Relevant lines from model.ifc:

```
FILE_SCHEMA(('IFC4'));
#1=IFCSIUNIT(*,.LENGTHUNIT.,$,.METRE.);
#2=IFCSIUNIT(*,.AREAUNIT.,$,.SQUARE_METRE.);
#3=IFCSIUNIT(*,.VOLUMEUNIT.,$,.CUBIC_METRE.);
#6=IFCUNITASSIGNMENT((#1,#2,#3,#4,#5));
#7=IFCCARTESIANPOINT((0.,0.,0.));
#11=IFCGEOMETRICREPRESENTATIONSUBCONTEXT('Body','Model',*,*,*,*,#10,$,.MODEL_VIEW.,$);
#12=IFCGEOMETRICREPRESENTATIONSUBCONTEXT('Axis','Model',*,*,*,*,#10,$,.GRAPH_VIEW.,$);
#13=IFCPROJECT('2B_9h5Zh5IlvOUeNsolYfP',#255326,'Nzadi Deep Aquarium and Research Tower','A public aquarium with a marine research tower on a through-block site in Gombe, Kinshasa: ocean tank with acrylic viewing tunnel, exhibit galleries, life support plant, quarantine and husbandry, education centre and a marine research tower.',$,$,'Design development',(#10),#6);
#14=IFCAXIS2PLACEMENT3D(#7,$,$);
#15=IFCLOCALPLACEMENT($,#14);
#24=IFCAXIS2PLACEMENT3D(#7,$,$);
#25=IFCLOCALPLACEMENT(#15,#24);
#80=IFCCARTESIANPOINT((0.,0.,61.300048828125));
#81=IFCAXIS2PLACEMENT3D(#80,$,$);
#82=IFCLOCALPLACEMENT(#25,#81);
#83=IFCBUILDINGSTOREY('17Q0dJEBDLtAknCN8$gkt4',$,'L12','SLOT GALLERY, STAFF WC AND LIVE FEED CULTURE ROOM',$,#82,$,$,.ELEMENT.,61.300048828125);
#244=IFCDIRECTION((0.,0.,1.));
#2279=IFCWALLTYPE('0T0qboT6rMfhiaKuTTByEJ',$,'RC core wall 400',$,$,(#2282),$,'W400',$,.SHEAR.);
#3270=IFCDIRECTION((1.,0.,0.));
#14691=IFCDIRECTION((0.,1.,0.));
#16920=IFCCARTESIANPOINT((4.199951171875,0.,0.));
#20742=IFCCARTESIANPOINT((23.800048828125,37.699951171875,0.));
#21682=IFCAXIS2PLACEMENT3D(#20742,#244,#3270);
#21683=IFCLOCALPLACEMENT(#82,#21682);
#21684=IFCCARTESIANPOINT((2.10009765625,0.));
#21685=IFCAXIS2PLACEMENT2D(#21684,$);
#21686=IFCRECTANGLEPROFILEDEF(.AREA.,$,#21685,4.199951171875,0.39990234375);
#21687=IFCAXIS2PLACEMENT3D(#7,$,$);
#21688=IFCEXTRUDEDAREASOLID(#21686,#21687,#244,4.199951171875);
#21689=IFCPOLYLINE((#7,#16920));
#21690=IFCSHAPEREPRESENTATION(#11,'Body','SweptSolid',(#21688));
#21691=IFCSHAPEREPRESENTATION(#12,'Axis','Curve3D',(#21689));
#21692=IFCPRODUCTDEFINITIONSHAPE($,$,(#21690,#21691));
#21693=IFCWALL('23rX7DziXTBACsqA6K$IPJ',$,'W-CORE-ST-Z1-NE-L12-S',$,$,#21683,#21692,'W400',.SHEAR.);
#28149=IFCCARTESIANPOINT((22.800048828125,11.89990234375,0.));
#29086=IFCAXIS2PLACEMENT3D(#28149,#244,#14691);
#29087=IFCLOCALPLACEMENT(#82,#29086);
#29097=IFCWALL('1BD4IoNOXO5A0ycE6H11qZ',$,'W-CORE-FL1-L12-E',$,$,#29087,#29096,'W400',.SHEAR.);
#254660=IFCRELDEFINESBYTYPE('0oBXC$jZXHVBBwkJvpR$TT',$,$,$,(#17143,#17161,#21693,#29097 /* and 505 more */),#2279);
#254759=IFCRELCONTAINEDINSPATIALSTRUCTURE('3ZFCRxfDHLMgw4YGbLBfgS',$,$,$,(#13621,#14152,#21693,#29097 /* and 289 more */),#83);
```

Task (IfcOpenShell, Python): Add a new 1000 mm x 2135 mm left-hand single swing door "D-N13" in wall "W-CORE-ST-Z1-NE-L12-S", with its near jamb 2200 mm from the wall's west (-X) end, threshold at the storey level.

```python
import numpy as np
import ifcopenshell
import ifcopenshell.api.feature
import ifcopenshell.api.geometry
import ifcopenshell.api.root
import ifcopenshell.api.spatial
import ifcopenshell.geom
import ifcopenshell.util.element
import ifcopenshell.util.placement
import ifcopenshell.util.representation
import ifcopenshell.util.shape
import ifcopenshell.util.unit

model = ifcopenshell.open("model.ifc")
unit_scale = ifcopenshell.util.unit.calculate_unit_scale(model)
settings = ifcopenshell.geom.settings()


def volume(element):
    """Net volume in cubic metres, openings subtracted."""
    shape = ifcopenshell.geom.create_shape(settings, element)
    return ifcopenshell.util.shape.get_volume(shape.geometry)


wall = model.by_guid("23rX7DziXTBACsqA6K$IPJ")
storey = ifcopenshell.util.element.get_container(wall, ifc_class="IfcBuildingStorey")
context = ifcopenshell.util.representation.get_context(model, "Model", "Body", "MODEL_VIEW")
before = volume(wall)

width, height, from_end, sill = 1, 2.135, 2.2, 0.0  # metres

# The wall runs along its own X axis, and the end named is its -X end.
wall_shape = ifcopenshell.geom.create_shape(settings, wall)
x, y, z = ifcopenshell.util.shape.get_vertices(wall_shape.geometry).T
start = x.min() + from_end
face, thickness = float(y.min()), float(y.max() - y.min())
wall_matrix = ifcopenshell.util.placement.get_local_placement(wall.ObjectPlacement)
level = ifcopenshell.util.placement.get_local_placement(storey.ObjectPlacement)[2, 3]


def in_wall(x, y):
    """Placement at x, y metres in the wall's axes, at sill height."""
    matrix = wall_matrix.copy()
    matrix[:, 3] = wall_matrix @ np.array([x / unit_scale, y / unit_scale, 0.0, 1.0])
    matrix[2, 3] = level + sill / unit_scale
    return matrix


# Opening: a box that overshoots both wall faces by 50 mm.
opening = ifcopenshell.api.root.create_entity(model, ifc_class="IfcOpeningElement", predefined_type="OPENING")
box = ifcopenshell.api.geometry.add_wall_representation(
    model, context=context, length=width, height=height, thickness=thickness + 0.1
)
ifcopenshell.api.geometry.assign_representation(model, product=opening, representation=box)
ifcopenshell.api.geometry.edit_object_placement(model, product=opening, matrix=in_wall(start, face - 0.05), is_si=False)
ifcopenshell.api.feature.add_feature(model, feature=opening, element=wall)

door = ifcopenshell.api.root.create_entity(model, ifc_class="IfcDoor", name="D-N13", predefined_type="DOOR")
door.OverallWidth, door.OverallHeight = width / unit_scale, height / unit_scale
door.OperationType = "SINGLE_SWING_LEFT"
body = ifcopenshell.api.geometry.add_door_representation(
    model,
    context=context,
    overall_width=door.OverallWidth,
    overall_height=door.OverallHeight,
    operation_type="SINGLE_SWING_LEFT",
    lining_properties={"LiningDepth": thickness / unit_scale, "ThresholdDepth": thickness / unit_scale},
)
ifcopenshell.api.geometry.assign_representation(model, product=door, representation=body)
ifcopenshell.api.spatial.assign_container(model, products=[door], relating_structure=storey)
ifcopenshell.api.feature.add_filling(model, opening=opening, element=door)

# The lining spans the wall, so the door starts at the wall face.
ifcopenshell.api.geometry.edit_object_placement(model, product=door, matrix=in_wall(start, face), is_si=False)

after = volume(wall)

print(f"wall volume {before:.3f} -> {after:.3f} m3")

model.write("model_rev.ifc")
```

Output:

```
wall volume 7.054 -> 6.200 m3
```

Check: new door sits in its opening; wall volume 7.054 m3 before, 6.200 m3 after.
